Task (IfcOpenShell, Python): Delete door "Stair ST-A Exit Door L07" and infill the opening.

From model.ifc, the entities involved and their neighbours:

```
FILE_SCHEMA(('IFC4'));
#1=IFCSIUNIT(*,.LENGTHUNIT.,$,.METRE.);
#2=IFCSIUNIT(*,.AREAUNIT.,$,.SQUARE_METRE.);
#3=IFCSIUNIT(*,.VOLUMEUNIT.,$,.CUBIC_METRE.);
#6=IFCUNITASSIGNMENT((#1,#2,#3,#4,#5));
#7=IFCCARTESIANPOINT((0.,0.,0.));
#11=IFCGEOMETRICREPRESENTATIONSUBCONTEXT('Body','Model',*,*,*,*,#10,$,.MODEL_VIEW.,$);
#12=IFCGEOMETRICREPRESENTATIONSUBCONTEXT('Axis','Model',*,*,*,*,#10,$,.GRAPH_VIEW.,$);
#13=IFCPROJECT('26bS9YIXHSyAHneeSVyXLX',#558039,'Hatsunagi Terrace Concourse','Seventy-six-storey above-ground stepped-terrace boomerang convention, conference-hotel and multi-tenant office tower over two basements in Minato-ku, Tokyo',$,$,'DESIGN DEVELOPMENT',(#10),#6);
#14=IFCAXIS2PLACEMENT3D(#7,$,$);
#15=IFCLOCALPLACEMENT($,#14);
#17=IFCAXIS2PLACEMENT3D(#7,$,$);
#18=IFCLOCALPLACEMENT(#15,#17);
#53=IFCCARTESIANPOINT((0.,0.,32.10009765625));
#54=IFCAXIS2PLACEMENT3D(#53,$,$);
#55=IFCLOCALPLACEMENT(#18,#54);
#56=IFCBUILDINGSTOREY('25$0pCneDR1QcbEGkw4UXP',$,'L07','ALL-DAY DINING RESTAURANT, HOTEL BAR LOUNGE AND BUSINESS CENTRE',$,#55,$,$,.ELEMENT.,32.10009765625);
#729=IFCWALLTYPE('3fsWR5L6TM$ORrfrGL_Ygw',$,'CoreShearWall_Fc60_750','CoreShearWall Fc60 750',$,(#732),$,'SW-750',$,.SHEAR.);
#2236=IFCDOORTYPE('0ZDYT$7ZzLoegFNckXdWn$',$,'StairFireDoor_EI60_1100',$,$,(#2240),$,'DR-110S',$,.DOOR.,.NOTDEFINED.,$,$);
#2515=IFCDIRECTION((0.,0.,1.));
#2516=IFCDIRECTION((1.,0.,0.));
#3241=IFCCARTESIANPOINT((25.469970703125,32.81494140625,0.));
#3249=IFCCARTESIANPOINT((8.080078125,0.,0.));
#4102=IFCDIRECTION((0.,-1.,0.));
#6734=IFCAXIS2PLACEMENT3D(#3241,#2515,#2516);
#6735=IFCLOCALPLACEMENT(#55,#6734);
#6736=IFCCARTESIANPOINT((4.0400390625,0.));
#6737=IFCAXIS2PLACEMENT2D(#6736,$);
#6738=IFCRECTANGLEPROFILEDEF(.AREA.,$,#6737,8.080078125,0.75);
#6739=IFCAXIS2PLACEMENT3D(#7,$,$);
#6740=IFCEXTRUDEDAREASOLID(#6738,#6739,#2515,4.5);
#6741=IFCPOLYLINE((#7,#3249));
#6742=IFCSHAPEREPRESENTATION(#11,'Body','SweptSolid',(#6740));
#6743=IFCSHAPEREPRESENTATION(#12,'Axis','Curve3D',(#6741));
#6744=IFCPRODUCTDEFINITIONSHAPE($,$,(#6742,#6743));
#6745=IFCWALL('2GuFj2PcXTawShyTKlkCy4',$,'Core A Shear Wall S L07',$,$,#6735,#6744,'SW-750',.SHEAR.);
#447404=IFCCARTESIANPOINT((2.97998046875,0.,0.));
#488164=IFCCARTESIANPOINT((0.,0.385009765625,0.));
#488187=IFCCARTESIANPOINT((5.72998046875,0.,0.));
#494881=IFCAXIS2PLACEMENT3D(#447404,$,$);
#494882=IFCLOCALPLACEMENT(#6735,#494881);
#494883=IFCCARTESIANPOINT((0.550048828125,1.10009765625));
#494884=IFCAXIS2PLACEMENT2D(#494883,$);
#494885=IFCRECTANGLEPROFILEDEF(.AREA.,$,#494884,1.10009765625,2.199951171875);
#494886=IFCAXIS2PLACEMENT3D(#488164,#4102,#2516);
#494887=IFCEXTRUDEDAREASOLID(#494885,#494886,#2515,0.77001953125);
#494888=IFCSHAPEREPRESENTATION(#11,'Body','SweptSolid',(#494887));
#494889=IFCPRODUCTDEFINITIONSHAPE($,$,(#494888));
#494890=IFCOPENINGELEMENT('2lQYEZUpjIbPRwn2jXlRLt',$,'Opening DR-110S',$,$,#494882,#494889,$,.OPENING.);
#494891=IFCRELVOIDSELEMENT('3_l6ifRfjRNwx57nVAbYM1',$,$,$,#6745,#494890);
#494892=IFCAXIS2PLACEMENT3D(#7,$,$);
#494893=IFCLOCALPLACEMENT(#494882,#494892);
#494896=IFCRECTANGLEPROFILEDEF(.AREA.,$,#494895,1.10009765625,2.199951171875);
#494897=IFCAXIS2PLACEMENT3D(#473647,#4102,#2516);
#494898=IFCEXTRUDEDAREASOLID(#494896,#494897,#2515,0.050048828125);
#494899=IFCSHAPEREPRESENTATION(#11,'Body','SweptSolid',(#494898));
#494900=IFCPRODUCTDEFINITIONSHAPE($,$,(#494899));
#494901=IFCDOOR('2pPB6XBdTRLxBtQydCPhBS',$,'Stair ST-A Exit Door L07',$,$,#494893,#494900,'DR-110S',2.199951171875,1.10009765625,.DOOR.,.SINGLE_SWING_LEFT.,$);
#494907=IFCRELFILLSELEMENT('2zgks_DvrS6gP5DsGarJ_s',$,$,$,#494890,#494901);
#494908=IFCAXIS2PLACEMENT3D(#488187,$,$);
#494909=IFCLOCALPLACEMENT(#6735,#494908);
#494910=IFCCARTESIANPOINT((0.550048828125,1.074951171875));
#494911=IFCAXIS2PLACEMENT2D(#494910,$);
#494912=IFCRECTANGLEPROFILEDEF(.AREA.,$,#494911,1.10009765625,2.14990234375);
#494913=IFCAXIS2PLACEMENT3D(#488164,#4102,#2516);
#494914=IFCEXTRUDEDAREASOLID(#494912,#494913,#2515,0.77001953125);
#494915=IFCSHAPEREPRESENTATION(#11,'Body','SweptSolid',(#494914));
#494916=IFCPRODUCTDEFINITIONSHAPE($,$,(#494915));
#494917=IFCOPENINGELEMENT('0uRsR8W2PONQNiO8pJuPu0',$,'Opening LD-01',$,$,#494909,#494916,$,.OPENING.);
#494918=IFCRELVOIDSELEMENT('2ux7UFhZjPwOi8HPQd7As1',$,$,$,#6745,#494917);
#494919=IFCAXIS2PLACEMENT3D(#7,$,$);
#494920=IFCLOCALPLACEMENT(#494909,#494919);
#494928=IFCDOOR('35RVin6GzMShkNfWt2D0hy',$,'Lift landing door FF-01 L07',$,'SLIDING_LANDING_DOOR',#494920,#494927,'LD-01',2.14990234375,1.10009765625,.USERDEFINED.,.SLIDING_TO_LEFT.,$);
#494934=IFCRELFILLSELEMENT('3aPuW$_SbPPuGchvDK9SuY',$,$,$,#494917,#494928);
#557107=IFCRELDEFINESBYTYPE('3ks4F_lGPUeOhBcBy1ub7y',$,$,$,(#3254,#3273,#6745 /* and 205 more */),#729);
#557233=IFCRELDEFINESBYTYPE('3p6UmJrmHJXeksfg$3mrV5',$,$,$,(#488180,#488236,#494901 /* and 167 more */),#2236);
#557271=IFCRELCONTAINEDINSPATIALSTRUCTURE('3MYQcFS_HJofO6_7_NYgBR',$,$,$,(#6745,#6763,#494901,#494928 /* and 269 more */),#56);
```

```python
import ifcopenshell
import ifcopenshell.api.feature
import ifcopenshell.api.root
import ifcopenshell.geom
import ifcopenshell.util.shape

model = ifcopenshell.open("model.ifc")
settings = ifcopenshell.geom.settings()


def volume(element):
    """Net volume in cubic metres, openings subtracted."""
    shape = ifcopenshell.geom.create_shape(settings, element)
    return ifcopenshell.util.shape.get_volume(shape.geometry)


door = model.by_id(494901)
opening = door.FillsVoids[0].RelatingOpeningElement
wall = opening.VoidsElements[0].RelatingBuildingElement
before = volume(wall)

ifcopenshell.api.root.remove_product(model, product=door)
ifcopenshell.api.feature.remove_feature(model, feature=opening)

after = volume(wall)

print(f"wall volume {before:.3f} -> {after:.3f} m3")

model.write("model_rev.ifc")
```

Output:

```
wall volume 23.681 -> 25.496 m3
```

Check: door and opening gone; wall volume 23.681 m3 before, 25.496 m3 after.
